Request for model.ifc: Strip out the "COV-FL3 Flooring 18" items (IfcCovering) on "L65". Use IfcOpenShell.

First a look at what the model holds.

```python
import ifcopenshell
import ifcopenshell.util.element

model = ifcopenshell.open("model.ifc")
print(model.schema)
storey = next(s for s in model.by_type("IfcBuildingStorey") if s.Name == "L65")
coverings = [e for e in ifcopenshell.util.element.get_decomposition(storey) if e.is_a("IfcCovering")]
seen = {}
for e in coverings:
    element_type = ifcopenshell.util.element.get_type(e)
    name = element_type.Name if element_type not in (None, e) else None
    seen[name] = seen.get(name, 0) + 1
for name, count in sorted(seen.items(), key=str):
    print(count, "x", name)
```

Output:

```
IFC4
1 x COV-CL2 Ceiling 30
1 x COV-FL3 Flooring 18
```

```python
import ifcopenshell
import ifcopenshell.api.root
import ifcopenshell.util.element

model = ifcopenshell.open("model.ifc")

storey = next(s for s in model.by_type("IfcBuildingStorey") if s.Name == "L65")
coverings = [e for e in ifcopenshell.util.element.get_decomposition(storey) if e.is_a("IfcCovering")]
targets = [e for e in coverings if (t := ifcopenshell.util.element.get_type(e)) not in (None, e) and t.Name == "COV-FL3 Flooring 18"]

for e in targets:
    ifcopenshell.api.root.remove_product(model, product=e)
print(len(targets), "removed")

model.write("model-out.ifc")
```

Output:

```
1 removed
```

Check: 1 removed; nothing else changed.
